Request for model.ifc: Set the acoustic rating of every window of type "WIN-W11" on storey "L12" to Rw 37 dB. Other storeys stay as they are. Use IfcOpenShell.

First a look at what the model holds.

```python
import ifcopenshell
import ifcopenshell.util.element

model = ifcopenshell.open("model.ifc")
print(model.schema)
storey = next(s for s in model.by_type("IfcBuildingStorey") if s.Name == "L12")
windows = [e for e in ifcopenshell.util.element.get_decomposition(storey) if e.is_a("IfcWindow")]
seen = {}
for e in windows:
    element_type = ifcopenshell.util.element.get_type(e)
    key = (element_type.Name if element_type != e and element_type else None, ifcopenshell.util.element.get_pset(e, "Pset_WindowCommon", "AcousticRating"))
    seen[key] = seen.get(key, 0) + 1
for (name, value), count in sorted(seen.items(), key=str):
    print(count, "x", name, "|", value)
```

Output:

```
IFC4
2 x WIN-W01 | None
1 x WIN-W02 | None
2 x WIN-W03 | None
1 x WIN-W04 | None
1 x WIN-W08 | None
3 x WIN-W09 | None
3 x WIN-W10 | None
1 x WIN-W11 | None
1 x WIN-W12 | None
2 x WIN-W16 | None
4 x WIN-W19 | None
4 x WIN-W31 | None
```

```python
import ifcopenshell
import ifcopenshell.api.pset
import ifcopenshell.util.element

model = ifcopenshell.open("model.ifc")

storey = next(s for s in model.by_type("IfcBuildingStorey") if s.Name == "L12")
windows = [e for e in ifcopenshell.util.element.get_decomposition(storey) if e.is_a("IfcWindow")]

count = 0
for e in windows:
    element_type = ifcopenshell.util.element.get_type(e)
    if element_type in (None, e) or element_type.Name != "WIN-W11":
        continue
    # add_pset returns the element's existing set when there is one.
    pset = ifcopenshell.api.pset.add_pset(model, product=e, name="Pset_WindowCommon")
    ifcopenshell.api.pset.edit_pset(model, pset=pset, properties={"AcousticRating": "Rw 37 dB"})
    count += 1

print(count, "windows updated")

model.write("model_edited.ifc")
```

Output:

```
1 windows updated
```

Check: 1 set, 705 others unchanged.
